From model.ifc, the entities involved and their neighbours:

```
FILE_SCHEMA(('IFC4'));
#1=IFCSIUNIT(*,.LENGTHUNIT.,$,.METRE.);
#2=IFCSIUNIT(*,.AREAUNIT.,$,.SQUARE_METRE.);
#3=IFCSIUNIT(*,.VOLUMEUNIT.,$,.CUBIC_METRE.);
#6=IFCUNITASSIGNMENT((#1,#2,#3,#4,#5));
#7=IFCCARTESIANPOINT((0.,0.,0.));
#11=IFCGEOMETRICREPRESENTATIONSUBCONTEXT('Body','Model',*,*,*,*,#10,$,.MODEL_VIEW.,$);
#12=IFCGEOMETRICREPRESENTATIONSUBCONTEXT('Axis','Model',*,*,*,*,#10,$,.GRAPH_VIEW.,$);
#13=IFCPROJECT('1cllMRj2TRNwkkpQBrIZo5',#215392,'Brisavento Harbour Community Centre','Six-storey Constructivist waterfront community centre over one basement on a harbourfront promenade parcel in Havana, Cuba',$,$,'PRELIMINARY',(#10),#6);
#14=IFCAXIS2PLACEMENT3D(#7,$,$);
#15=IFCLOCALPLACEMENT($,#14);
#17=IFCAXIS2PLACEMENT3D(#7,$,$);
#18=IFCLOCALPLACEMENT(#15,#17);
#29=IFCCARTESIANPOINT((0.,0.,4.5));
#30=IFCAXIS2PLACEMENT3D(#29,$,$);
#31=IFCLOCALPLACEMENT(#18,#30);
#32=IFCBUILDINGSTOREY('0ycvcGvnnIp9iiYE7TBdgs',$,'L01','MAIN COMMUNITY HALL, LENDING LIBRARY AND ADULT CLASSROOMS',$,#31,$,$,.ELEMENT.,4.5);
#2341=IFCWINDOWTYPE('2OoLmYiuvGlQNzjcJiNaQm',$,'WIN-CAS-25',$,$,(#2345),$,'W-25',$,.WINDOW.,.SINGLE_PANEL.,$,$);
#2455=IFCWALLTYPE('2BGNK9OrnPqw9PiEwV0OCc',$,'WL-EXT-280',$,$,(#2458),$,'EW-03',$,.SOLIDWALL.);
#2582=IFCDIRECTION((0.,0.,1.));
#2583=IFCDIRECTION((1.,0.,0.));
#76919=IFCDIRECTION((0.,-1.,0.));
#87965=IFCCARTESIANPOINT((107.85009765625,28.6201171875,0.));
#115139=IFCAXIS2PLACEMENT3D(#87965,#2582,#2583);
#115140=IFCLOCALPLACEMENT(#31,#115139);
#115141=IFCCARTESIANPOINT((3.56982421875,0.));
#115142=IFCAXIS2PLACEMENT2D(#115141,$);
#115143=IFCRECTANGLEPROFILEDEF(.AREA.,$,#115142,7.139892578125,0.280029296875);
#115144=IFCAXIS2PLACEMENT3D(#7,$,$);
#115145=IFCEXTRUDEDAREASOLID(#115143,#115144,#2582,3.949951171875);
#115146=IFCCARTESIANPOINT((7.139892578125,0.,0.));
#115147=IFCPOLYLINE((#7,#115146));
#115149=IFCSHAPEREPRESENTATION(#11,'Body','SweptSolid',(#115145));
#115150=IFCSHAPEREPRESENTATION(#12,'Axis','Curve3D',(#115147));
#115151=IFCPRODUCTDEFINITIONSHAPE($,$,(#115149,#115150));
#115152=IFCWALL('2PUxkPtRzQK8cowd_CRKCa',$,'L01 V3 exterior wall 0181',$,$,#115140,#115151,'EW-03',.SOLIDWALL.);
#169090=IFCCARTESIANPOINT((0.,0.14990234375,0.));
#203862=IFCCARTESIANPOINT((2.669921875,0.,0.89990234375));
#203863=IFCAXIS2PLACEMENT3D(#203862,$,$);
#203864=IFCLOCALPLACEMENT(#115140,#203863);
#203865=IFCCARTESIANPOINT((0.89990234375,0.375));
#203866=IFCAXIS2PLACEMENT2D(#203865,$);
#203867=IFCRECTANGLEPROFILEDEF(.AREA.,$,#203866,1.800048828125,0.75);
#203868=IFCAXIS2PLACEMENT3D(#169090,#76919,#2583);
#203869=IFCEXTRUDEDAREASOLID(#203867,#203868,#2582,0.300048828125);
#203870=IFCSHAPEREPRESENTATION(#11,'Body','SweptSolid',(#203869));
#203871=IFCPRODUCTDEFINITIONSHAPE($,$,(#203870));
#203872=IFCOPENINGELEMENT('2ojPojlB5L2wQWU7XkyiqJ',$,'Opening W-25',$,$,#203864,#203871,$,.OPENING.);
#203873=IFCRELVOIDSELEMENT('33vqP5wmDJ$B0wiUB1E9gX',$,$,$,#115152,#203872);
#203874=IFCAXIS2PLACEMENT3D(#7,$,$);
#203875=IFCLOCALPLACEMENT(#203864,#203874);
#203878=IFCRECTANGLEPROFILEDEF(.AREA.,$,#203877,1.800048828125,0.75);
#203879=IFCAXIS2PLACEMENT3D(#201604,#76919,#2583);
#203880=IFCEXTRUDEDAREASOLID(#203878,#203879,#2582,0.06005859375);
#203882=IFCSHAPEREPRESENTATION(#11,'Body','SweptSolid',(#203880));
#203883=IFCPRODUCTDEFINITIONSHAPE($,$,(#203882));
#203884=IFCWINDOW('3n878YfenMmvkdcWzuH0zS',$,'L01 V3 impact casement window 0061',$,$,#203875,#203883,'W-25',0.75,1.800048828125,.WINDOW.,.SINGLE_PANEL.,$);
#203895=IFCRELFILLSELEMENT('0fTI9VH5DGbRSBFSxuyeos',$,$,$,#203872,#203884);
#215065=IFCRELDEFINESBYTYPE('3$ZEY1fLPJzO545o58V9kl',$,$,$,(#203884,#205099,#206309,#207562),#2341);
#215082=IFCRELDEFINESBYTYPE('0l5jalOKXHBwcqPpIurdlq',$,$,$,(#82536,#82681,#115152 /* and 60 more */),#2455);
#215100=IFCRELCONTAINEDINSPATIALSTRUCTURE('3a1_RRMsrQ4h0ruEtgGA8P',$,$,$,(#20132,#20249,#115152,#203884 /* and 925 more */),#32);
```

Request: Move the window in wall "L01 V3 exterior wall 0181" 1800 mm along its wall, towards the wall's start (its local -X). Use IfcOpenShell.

```python
import ifcopenshell
import ifcopenshell.api.geometry
import ifcopenshell.util.placement

model = ifcopenshell.open("model.ifc")

window = model.by_guid("3n878YfenMmvkdcWzuH0zS")
opening = window.FillsVoids[0].RelatingOpeningElement
wall = opening.VoidsElements[0].RelatingBuildingElement

wall_matrix = ifcopenshell.util.placement.get_local_placement(wall.ObjectPlacement)
shift = wall_matrix[:3, 0] * -1.8
before = ifcopenshell.util.placement.get_local_placement(window.ObjectPlacement)[:3, 3].copy()

# The window is placed relative to its opening, so it follows when the opening moves.
matrix = ifcopenshell.util.placement.get_local_placement(opening.ObjectPlacement)
matrix[:3, 3] += shift
ifcopenshell.api.geometry.edit_object_placement(
    model, product=opening, matrix=matrix, is_si=False, should_transform_children=True
)

after = ifcopenshell.util.placement.get_local_placement(window.ObjectPlacement)[:3, 3]
print("window moved by", (after - before).round(3) + 0.0)

model.write("model_updated.ifc")
```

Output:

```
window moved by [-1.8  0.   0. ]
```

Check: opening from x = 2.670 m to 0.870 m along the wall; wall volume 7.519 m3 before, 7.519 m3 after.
